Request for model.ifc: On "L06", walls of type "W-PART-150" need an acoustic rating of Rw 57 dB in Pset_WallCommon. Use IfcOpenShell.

First a look at what the model holds.

```python
import ifcopenshell
import ifcopenshell.util.element

model = ifcopenshell.open("model.ifc")
print(model.schema)
storey = next(s for s in model.by_type("IfcBuildingStorey") if s.Name == "L06")
walls = [e for e in ifcopenshell.util.element.get_decomposition(storey) if e.is_a("IfcWall")]
seen = {}
for e in walls:
    element_type = ifcopenshell.util.element.get_type(e)
    key = (element_type.Name if element_type != e and element_type else None, ifcopenshell.util.element.get_pset(e, "Pset_WallCommon", "AcousticRating"))
    seen[key] = seen.get(key, 0) + 1
for (name, value), count in sorted(seen.items(), key=str):
    print(count, "x", name, "|", value)
```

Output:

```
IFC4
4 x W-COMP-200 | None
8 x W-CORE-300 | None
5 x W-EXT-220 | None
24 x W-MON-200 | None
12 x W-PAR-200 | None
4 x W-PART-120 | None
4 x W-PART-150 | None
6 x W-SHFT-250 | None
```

```python
import ifcopenshell
import ifcopenshell.api.pset
import ifcopenshell.util.element

model = ifcopenshell.open("model.ifc")

storey = next(s for s in model.by_type("IfcBuildingStorey") if s.Name == "L06")
walls = [e for e in ifcopenshell.util.element.get_decomposition(storey) if e.is_a("IfcWall")]

count = 0
for e in walls:
    element_type = ifcopenshell.util.element.get_type(e)
    if element_type in (None, e) or element_type.Name != "W-PART-150":
        continue
    # add_pset returns the element's existing set when there is one.
    pset = ifcopenshell.api.pset.add_pset(model, product=e, name="Pset_WallCommon")
    ifcopenshell.api.pset.edit_pset(model, pset=pset, properties={"AcousticRating": "Rw 57 dB"})
    count += 1

print(count, "walls updated")

model.write("model_edited.ifc")
```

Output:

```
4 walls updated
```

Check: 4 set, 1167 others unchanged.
